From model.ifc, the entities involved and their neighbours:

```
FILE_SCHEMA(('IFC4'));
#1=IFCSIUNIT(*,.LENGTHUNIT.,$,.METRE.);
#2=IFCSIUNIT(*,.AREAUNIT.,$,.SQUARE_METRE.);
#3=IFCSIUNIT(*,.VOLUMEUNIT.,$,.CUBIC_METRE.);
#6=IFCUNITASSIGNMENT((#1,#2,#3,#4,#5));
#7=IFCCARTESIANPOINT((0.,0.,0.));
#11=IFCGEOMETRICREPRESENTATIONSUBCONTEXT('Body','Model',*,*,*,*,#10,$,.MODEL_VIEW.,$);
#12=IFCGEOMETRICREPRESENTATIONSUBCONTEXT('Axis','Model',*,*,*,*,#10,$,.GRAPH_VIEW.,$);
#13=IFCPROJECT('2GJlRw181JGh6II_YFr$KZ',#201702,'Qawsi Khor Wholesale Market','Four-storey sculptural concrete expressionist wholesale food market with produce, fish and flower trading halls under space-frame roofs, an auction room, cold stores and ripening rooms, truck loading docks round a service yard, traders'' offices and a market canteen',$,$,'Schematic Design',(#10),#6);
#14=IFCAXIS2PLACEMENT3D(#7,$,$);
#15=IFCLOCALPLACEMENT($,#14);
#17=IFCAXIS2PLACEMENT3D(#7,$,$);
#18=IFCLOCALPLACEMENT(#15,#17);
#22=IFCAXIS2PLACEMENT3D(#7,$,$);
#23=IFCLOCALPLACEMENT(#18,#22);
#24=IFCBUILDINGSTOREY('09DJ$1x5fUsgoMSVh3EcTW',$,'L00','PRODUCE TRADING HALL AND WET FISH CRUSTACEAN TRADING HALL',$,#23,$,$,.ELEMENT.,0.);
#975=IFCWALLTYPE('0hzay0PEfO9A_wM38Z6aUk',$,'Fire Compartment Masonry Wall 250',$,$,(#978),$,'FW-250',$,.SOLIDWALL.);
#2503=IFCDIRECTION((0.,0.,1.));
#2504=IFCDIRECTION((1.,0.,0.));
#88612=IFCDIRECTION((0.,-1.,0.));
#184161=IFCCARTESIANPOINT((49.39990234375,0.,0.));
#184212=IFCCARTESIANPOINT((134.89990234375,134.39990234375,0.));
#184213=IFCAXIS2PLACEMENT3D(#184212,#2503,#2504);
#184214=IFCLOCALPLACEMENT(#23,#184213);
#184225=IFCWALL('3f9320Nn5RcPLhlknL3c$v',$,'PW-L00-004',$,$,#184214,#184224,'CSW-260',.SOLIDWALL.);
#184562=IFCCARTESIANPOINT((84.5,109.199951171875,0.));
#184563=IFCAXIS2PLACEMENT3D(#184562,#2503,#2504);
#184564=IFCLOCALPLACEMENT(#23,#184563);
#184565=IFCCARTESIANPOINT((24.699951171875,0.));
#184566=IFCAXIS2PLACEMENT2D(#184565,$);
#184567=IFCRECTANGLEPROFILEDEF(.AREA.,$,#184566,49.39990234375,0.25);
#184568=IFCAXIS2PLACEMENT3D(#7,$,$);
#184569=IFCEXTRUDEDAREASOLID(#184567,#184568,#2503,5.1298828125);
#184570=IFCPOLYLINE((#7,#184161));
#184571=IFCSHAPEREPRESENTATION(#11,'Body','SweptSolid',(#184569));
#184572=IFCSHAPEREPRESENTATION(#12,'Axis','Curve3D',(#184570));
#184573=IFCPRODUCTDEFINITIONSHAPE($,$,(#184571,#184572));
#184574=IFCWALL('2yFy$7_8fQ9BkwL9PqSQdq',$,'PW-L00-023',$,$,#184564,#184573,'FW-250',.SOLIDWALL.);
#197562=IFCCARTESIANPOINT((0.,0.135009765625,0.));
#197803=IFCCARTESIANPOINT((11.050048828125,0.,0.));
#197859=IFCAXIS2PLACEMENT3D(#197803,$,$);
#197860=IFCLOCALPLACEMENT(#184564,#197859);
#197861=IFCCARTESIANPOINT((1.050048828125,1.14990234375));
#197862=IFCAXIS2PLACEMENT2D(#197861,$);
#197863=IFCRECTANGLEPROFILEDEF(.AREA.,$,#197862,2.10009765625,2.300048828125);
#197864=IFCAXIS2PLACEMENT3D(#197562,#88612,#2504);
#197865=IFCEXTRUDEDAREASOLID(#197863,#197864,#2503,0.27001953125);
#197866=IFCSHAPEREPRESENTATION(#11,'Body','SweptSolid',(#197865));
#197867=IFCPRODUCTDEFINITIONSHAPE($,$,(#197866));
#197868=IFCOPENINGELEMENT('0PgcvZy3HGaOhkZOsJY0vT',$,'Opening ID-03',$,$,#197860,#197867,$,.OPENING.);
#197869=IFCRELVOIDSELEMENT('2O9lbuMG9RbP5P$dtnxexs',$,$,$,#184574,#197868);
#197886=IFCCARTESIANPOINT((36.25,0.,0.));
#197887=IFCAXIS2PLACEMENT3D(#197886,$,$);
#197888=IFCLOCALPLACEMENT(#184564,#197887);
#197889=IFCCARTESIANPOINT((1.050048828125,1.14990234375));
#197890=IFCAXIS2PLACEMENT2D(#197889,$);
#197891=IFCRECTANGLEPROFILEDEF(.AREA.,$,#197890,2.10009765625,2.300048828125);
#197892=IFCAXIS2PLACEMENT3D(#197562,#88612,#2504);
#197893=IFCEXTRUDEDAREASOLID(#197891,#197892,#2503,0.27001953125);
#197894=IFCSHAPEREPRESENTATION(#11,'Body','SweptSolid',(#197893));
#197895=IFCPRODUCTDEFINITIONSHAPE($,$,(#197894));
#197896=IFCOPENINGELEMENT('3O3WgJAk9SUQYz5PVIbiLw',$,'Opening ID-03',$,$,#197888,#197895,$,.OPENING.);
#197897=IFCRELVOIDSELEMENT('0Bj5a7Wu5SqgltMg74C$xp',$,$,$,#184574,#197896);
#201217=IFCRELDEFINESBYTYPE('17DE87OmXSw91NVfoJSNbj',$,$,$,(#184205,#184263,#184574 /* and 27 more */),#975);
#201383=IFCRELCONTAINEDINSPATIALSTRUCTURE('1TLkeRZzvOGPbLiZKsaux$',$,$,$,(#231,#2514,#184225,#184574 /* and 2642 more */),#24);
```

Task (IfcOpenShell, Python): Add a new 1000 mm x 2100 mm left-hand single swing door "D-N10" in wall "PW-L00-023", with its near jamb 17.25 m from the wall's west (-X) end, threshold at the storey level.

```python
import numpy as np
import ifcopenshell
import ifcopenshell.api.feature
import ifcopenshell.api.geometry
import ifcopenshell.api.root
import ifcopenshell.api.spatial
import ifcopenshell.geom
import ifcopenshell.util.element
import ifcopenshell.util.placement
import ifcopenshell.util.representation
import ifcopenshell.util.shape
import ifcopenshell.util.unit

model = ifcopenshell.open("model.ifc")
unit_scale = ifcopenshell.util.unit.calculate_unit_scale(model)
settings = ifcopenshell.geom.settings()


def volume(element):
    """Net volume in cubic metres, openings subtracted."""
    shape = ifcopenshell.geom.create_shape(settings, element)
    return ifcopenshell.util.shape.get_volume(shape.geometry)


wall = model.by_guid("2yFy$7_8fQ9BkwL9PqSQdq")
storey = ifcopenshell.util.element.get_container(wall, ifc_class="IfcBuildingStorey")
context = ifcopenshell.util.representation.get_context(model, "Model", "Body", "MODEL_VIEW")
before = volume(wall)

width, height, from_end, sill = 1, 2.1, 17.25, 0.0  # metres

# The wall runs along its own X axis, and the end named is its -X end.
wall_shape = ifcopenshell.geom.create_shape(settings, wall)
x, y, z = ifcopenshell.util.shape.get_vertices(wall_shape.geometry).T
start = x.min() + from_end
face, thickness = float(y.min()), float(y.max() - y.min())
wall_matrix = ifcopenshell.util.placement.get_local_placement(wall.ObjectPlacement)
level = ifcopenshell.util.placement.get_local_placement(storey.ObjectPlacement)[2, 3]


def in_wall(x, y):
    """Placement at x, y metres in the wall's axes, at sill height."""
    matrix = wall_matrix.copy()
    matrix[:, 3] = wall_matrix @ np.array([x / unit_scale, y / unit_scale, 0.0, 1.0])
    matrix[2, 3] = level + sill / unit_scale
    return matrix


# Opening: a box that overshoots both wall faces by 50 mm.
opening = ifcopenshell.api.root.create_entity(model, ifc_class="IfcOpeningElement", predefined_type="OPENING")
box = ifcopenshell.api.geometry.add_wall_representation(
    model, context=context, length=width, height=height, thickness=thickness + 0.1
)
ifcopenshell.api.geometry.assign_representation(model, product=opening, representation=box)
ifcopenshell.api.geometry.edit_object_placement(model, product=opening, matrix=in_wall(start, face - 0.05), is_si=False)
ifcopenshell.api.feature.add_feature(model, feature=opening, element=wall)

door = ifcopenshell.api.root.create_entity(model, ifc_class="IfcDoor", name="D-N10", predefined_type="DOOR")
door.OverallWidth, door.OverallHeight = width / unit_scale, height / unit_scale
door.OperationType = "SINGLE_SWING_LEFT"
body = ifcopenshell.api.geometry.add_door_representation(
    model,
    context=context,
    overall_width=door.OverallWidth,
    overall_height=door.OverallHeight,
    operation_type="SINGLE_SWING_LEFT",
    lining_properties={"LiningDepth": thickness / unit_scale, "ThresholdDepth": thickness / unit_scale},
)
ifcopenshell.api.geometry.assign_representation(model, product=door, representation=body)
ifcopenshell.api.spatial.assign_container(model, products=[door], relating_structure=storey)
ifcopenshell.api.feature.add_filling(model, opening=opening, element=door)

# The lining spans the wall, so the door starts at the wall face.
ifcopenshell.api.geometry.edit_object_placement(model, product=door, matrix=in_wall(start, face), is_si=False)

after = volume(wall)

print(f"wall volume {before:.3f} -> {after:.3f} m3")

model.write("model_rev.ifc")
```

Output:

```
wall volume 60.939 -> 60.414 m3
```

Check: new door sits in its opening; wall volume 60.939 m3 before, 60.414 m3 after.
